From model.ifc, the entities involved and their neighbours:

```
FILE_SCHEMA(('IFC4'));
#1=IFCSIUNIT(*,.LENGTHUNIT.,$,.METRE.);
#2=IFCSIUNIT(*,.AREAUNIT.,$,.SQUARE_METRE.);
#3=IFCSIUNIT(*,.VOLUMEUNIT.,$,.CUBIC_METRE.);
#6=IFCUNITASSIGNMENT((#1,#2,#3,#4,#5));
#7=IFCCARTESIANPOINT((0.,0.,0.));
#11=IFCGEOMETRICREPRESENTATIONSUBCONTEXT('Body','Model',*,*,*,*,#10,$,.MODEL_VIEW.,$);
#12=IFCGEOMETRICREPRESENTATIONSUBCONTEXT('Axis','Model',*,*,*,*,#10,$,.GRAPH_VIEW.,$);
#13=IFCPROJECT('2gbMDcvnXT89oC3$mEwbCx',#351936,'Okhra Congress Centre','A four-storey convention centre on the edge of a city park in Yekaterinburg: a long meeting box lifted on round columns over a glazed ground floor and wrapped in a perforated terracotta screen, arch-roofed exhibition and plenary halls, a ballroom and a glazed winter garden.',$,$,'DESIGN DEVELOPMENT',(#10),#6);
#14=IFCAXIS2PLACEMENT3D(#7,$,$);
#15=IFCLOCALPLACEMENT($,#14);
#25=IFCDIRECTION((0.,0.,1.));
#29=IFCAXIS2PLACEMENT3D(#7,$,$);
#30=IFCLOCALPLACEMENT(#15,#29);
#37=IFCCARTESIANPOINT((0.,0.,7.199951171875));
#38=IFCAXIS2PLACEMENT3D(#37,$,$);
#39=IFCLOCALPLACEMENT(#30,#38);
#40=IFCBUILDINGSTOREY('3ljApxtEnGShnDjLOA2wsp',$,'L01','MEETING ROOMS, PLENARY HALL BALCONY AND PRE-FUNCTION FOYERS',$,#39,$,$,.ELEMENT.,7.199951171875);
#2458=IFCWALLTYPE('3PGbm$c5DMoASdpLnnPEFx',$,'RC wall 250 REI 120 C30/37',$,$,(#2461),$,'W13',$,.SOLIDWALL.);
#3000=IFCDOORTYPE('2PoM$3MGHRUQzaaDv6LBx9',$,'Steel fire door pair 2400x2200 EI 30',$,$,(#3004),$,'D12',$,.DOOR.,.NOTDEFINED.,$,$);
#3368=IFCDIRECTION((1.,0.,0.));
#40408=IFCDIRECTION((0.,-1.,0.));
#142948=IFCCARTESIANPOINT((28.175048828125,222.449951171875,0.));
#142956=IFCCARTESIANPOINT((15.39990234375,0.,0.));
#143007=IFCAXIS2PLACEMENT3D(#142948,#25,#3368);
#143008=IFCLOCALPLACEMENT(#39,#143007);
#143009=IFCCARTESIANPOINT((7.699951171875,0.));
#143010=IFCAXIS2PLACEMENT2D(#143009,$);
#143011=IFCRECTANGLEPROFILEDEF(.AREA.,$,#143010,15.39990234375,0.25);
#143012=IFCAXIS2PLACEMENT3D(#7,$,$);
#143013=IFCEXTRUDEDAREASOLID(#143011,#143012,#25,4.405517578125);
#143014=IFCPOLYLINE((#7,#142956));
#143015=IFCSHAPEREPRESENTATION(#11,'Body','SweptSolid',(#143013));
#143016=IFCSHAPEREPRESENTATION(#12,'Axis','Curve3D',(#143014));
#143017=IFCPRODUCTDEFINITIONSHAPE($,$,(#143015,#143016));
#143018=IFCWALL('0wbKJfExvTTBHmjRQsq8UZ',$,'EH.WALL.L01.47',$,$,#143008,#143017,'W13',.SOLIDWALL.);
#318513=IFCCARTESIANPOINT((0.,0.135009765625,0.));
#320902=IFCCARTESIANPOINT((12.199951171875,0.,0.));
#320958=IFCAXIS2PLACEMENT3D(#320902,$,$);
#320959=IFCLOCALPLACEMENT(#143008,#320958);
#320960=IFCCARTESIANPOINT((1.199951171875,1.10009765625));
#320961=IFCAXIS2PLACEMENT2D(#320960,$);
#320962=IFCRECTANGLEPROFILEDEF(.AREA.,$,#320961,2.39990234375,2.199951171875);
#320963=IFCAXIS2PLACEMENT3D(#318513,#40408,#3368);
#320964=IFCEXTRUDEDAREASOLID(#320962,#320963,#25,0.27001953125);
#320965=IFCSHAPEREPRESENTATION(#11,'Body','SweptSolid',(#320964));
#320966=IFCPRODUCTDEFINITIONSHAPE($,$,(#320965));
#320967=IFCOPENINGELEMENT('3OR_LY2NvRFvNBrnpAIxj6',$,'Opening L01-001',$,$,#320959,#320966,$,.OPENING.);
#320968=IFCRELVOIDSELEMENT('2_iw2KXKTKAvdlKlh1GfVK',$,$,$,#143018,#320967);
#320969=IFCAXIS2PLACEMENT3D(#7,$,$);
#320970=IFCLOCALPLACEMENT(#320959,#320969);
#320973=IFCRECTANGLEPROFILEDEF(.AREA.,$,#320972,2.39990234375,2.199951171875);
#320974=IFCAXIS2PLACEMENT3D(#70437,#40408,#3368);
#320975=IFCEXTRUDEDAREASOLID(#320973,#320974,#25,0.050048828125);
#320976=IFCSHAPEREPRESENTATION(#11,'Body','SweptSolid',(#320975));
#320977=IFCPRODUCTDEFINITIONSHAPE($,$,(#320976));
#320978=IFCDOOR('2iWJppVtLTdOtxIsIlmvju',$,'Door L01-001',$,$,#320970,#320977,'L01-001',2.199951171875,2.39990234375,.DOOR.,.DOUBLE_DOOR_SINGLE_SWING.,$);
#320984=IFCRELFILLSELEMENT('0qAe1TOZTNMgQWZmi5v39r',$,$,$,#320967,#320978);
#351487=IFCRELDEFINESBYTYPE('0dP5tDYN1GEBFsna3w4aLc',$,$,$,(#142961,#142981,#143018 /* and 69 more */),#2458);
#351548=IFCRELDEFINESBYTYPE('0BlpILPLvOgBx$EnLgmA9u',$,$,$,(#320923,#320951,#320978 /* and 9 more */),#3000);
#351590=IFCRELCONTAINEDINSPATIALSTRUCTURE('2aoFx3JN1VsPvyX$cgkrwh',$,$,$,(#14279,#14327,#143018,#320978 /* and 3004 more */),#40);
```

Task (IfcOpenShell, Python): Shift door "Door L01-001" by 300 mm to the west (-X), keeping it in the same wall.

```python
import ifcopenshell
import ifcopenshell.api.geometry
import ifcopenshell.util.placement
import ifcopenshell.util.unit

model = ifcopenshell.open("model.ifc")
unit_scale = ifcopenshell.util.unit.calculate_unit_scale(model)

door = model.by_guid("2iWJppVtLTdOtxIsIlmvju")
opening = door.FillsVoids[0].RelatingOpeningElement
wall = opening.VoidsElements[0].RelatingBuildingElement

wall_matrix = ifcopenshell.util.placement.get_local_placement(wall.ObjectPlacement)
shift = wall_matrix[:3, 0] * -0.3 / unit_scale
before = ifcopenshell.util.placement.get_local_placement(door.ObjectPlacement)[:3, 3].copy()

# The door is placed relative to its opening, so it follows when the opening moves.
matrix = ifcopenshell.util.placement.get_local_placement(opening.ObjectPlacement)
matrix[:3, 3] += shift
ifcopenshell.api.geometry.edit_object_placement(
    model, product=opening, matrix=matrix, is_si=False, should_transform_children=True
)

after = ifcopenshell.util.placement.get_local_placement(door.ObjectPlacement)[:3, 3]
print("door moved by", (after - before).round(3) + 0.0)

model.write("model-out.ifc")
```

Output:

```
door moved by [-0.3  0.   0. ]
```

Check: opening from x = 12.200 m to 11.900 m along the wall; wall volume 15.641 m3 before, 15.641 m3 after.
